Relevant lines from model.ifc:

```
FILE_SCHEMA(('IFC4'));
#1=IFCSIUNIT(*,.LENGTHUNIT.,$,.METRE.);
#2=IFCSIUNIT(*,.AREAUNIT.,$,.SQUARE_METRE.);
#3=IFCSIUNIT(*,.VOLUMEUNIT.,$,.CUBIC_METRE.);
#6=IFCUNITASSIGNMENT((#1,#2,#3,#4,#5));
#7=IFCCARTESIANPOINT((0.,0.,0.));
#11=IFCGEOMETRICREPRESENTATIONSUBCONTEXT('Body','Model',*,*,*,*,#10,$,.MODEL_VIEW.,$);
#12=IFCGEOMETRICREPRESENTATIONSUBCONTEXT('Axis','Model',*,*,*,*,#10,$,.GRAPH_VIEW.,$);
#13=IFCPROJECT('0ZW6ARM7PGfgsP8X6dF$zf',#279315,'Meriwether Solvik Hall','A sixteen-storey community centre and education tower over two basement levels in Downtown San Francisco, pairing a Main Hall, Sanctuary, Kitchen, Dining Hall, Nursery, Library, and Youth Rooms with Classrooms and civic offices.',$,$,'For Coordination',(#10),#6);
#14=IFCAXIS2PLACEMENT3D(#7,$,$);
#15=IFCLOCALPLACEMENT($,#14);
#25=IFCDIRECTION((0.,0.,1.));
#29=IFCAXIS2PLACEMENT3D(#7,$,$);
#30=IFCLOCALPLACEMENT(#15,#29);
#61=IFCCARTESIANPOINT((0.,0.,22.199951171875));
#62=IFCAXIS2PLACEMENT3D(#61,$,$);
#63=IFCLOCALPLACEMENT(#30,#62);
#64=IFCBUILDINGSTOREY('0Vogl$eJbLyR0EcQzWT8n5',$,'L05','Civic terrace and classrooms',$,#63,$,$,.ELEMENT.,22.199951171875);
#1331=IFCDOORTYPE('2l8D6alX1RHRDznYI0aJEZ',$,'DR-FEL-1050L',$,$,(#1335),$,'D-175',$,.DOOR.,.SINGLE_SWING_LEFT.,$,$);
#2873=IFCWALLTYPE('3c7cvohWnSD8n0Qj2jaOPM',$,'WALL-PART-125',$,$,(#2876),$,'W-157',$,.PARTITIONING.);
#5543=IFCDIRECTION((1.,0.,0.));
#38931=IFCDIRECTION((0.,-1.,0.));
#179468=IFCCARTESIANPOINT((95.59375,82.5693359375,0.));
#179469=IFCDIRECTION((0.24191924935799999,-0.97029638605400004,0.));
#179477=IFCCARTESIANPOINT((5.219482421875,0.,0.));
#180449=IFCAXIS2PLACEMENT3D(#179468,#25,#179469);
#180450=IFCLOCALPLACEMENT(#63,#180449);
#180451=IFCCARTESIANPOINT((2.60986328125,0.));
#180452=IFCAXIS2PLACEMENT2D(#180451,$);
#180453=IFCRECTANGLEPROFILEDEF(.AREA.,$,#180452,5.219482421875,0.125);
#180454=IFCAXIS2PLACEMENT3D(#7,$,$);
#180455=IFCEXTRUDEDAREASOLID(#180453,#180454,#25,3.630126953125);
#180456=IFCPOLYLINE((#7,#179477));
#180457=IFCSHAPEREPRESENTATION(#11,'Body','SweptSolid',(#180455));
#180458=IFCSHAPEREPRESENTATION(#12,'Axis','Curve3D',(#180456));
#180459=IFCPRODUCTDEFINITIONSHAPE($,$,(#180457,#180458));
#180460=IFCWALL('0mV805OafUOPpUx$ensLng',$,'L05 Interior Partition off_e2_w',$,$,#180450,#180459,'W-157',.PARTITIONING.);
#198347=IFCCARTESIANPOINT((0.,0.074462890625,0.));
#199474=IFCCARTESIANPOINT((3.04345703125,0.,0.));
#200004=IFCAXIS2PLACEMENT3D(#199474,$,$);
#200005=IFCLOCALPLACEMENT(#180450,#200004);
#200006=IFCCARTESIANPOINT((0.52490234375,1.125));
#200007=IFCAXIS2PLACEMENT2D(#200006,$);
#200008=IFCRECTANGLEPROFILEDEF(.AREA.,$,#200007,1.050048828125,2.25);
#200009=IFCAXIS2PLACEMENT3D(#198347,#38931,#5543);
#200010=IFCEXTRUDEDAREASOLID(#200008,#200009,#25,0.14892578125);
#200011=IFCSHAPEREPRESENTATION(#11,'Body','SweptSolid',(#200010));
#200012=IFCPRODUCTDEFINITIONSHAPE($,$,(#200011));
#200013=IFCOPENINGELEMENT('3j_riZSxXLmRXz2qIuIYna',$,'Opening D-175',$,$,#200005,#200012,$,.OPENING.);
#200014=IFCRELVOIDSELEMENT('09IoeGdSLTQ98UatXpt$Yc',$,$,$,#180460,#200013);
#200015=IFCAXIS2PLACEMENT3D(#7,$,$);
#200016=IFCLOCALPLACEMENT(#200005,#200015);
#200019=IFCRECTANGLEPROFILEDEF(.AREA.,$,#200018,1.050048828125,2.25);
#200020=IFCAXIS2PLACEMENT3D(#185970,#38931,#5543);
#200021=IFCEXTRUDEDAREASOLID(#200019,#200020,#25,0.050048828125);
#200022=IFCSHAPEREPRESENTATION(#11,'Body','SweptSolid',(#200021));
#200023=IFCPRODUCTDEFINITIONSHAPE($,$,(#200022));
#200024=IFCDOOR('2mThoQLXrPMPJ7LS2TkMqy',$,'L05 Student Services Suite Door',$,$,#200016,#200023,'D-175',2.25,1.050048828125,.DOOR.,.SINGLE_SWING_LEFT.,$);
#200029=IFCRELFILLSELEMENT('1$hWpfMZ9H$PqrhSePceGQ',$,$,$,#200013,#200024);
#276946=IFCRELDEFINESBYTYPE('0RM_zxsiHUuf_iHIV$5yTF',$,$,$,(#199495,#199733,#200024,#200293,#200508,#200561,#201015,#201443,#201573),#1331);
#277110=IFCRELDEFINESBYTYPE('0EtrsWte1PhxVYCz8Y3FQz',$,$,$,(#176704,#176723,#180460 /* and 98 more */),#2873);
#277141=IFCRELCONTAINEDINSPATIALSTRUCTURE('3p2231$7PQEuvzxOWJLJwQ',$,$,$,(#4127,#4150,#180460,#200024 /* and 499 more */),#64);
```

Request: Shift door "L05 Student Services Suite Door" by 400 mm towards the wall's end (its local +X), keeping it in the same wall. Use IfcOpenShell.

```python
import ifcopenshell
import ifcopenshell.api.geometry
import ifcopenshell.util.placement
import ifcopenshell.util.unit

model = ifcopenshell.open("model.ifc")
unit_scale = ifcopenshell.util.unit.calculate_unit_scale(model)

door = model.by_guid("2mThoQLXrPMPJ7LS2TkMqy")
opening = door.FillsVoids[0].RelatingOpeningElement
wall = opening.VoidsElements[0].RelatingBuildingElement

wall_matrix = ifcopenshell.util.placement.get_local_placement(wall.ObjectPlacement)
shift = wall_matrix[:3, 0] * 0.4 / unit_scale
before = ifcopenshell.util.placement.get_local_placement(door.ObjectPlacement)[:3, 3].copy()

# The door is placed relative to its opening, so it follows when the opening moves.
matrix = ifcopenshell.util.placement.get_local_placement(opening.ObjectPlacement)
matrix[:3, 3] += shift
ifcopenshell.api.geometry.edit_object_placement(
    model, product=opening, matrix=matrix, is_si=False, should_transform_children=True
)

after = ifcopenshell.util.placement.get_local_placement(door.ObjectPlacement)[:3, 3]
print("door moved by", (after - before).round(3) + 0.0)

model.write("model_updated.ifc")
```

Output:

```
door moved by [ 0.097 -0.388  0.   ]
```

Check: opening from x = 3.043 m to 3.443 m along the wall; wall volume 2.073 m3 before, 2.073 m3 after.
